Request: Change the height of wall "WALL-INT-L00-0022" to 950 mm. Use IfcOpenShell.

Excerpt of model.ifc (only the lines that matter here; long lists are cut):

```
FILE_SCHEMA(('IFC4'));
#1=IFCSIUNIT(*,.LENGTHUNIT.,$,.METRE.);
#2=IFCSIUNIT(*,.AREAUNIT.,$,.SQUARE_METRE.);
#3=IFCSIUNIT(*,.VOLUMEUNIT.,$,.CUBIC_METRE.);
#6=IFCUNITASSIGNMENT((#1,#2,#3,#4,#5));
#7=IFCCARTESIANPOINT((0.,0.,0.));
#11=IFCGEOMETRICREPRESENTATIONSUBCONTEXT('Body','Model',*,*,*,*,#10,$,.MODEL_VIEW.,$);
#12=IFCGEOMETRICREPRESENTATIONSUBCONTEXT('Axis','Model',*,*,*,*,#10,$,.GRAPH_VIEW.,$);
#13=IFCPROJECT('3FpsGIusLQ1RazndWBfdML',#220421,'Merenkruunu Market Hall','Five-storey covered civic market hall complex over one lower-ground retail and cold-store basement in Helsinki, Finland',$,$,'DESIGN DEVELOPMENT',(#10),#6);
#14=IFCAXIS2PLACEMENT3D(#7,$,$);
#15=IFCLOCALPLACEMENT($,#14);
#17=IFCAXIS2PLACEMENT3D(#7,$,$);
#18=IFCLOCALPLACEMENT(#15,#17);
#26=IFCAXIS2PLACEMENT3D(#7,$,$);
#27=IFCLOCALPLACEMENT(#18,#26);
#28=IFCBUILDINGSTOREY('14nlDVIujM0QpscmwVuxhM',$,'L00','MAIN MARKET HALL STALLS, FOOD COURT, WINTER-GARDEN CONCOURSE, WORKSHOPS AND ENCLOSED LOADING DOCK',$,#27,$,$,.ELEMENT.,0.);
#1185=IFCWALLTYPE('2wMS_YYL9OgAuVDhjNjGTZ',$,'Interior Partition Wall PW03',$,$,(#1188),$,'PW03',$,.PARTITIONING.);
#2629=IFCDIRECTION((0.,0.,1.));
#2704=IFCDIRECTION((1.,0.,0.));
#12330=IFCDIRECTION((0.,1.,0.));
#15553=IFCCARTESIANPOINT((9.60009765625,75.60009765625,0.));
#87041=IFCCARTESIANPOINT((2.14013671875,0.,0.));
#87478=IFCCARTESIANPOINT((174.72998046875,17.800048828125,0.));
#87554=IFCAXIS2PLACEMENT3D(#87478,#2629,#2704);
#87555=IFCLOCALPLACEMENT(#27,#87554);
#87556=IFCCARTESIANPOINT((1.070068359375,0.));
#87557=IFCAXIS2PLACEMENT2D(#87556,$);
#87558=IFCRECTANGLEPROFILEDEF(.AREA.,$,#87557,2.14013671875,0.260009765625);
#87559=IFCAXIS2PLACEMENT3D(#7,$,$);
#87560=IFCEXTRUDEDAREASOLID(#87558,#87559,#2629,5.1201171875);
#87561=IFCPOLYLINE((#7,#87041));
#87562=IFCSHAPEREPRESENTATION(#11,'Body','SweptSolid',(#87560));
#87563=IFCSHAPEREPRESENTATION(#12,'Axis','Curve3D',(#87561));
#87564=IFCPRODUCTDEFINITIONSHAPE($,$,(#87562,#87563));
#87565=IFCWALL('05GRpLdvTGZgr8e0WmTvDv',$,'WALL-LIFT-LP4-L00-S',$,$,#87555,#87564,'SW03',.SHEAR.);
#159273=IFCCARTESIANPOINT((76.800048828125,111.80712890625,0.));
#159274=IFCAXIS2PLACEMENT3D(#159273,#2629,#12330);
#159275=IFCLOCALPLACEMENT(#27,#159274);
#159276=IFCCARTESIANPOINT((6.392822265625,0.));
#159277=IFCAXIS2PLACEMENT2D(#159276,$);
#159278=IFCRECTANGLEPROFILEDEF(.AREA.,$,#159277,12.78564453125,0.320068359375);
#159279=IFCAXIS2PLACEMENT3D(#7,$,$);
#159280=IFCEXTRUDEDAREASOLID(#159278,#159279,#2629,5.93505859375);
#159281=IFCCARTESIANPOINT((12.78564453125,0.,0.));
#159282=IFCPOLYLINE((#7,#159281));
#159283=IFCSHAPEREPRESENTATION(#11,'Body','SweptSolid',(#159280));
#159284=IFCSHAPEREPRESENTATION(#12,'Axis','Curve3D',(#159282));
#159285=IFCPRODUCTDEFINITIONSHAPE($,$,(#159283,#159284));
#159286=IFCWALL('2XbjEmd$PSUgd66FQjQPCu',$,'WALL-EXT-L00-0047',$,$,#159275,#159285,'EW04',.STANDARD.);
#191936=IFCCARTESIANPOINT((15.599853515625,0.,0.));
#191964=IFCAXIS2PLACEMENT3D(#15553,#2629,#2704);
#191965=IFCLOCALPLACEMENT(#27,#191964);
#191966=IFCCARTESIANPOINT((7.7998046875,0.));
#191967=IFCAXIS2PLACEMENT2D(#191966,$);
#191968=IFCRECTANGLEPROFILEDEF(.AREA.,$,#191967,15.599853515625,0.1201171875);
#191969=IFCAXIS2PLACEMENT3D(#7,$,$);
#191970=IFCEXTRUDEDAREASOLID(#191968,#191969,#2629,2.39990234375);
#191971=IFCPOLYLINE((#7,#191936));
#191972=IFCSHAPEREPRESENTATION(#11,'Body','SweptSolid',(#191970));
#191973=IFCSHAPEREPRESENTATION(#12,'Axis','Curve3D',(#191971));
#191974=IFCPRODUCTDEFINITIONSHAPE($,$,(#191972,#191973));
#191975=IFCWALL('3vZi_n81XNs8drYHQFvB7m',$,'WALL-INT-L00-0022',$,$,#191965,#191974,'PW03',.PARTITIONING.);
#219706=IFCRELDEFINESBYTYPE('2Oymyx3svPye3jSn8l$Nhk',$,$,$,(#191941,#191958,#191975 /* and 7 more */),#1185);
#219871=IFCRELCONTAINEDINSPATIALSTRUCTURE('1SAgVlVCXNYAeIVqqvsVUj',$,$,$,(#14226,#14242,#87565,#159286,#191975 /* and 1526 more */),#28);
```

```python
import ifcopenshell
import ifcopenshell.geom
import ifcopenshell.util.representation
import ifcopenshell.util.shape
import ifcopenshell.util.unit

model = ifcopenshell.open("model.ifc")
unit_scale = ifcopenshell.util.unit.calculate_unit_scale(model)
settings = ifcopenshell.geom.settings()


def volume(element):
    """Net volume in cubic metres, openings subtracted."""
    shape = ifcopenshell.geom.create_shape(settings, element)
    return ifcopenshell.util.shape.get_volume(shape.geometry)


wall = model.by_guid("3vZi_n81XNs8drYHQFvB7m")
before = volume(wall)

body = ifcopenshell.util.representation.get_representation(wall, "Model", "Body")
solid = body.Items[0]
old_height = solid.Depth
solid.Depth = 0.95 / unit_scale
after = volume(wall)

print(f"height {old_height:g} -> {solid.Depth:g}, volume {before:.3f} -> {after:.3f} m3")

model.write("model_rev.ifc")
```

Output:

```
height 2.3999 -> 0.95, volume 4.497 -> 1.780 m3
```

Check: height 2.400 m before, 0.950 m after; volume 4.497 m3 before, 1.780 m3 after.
